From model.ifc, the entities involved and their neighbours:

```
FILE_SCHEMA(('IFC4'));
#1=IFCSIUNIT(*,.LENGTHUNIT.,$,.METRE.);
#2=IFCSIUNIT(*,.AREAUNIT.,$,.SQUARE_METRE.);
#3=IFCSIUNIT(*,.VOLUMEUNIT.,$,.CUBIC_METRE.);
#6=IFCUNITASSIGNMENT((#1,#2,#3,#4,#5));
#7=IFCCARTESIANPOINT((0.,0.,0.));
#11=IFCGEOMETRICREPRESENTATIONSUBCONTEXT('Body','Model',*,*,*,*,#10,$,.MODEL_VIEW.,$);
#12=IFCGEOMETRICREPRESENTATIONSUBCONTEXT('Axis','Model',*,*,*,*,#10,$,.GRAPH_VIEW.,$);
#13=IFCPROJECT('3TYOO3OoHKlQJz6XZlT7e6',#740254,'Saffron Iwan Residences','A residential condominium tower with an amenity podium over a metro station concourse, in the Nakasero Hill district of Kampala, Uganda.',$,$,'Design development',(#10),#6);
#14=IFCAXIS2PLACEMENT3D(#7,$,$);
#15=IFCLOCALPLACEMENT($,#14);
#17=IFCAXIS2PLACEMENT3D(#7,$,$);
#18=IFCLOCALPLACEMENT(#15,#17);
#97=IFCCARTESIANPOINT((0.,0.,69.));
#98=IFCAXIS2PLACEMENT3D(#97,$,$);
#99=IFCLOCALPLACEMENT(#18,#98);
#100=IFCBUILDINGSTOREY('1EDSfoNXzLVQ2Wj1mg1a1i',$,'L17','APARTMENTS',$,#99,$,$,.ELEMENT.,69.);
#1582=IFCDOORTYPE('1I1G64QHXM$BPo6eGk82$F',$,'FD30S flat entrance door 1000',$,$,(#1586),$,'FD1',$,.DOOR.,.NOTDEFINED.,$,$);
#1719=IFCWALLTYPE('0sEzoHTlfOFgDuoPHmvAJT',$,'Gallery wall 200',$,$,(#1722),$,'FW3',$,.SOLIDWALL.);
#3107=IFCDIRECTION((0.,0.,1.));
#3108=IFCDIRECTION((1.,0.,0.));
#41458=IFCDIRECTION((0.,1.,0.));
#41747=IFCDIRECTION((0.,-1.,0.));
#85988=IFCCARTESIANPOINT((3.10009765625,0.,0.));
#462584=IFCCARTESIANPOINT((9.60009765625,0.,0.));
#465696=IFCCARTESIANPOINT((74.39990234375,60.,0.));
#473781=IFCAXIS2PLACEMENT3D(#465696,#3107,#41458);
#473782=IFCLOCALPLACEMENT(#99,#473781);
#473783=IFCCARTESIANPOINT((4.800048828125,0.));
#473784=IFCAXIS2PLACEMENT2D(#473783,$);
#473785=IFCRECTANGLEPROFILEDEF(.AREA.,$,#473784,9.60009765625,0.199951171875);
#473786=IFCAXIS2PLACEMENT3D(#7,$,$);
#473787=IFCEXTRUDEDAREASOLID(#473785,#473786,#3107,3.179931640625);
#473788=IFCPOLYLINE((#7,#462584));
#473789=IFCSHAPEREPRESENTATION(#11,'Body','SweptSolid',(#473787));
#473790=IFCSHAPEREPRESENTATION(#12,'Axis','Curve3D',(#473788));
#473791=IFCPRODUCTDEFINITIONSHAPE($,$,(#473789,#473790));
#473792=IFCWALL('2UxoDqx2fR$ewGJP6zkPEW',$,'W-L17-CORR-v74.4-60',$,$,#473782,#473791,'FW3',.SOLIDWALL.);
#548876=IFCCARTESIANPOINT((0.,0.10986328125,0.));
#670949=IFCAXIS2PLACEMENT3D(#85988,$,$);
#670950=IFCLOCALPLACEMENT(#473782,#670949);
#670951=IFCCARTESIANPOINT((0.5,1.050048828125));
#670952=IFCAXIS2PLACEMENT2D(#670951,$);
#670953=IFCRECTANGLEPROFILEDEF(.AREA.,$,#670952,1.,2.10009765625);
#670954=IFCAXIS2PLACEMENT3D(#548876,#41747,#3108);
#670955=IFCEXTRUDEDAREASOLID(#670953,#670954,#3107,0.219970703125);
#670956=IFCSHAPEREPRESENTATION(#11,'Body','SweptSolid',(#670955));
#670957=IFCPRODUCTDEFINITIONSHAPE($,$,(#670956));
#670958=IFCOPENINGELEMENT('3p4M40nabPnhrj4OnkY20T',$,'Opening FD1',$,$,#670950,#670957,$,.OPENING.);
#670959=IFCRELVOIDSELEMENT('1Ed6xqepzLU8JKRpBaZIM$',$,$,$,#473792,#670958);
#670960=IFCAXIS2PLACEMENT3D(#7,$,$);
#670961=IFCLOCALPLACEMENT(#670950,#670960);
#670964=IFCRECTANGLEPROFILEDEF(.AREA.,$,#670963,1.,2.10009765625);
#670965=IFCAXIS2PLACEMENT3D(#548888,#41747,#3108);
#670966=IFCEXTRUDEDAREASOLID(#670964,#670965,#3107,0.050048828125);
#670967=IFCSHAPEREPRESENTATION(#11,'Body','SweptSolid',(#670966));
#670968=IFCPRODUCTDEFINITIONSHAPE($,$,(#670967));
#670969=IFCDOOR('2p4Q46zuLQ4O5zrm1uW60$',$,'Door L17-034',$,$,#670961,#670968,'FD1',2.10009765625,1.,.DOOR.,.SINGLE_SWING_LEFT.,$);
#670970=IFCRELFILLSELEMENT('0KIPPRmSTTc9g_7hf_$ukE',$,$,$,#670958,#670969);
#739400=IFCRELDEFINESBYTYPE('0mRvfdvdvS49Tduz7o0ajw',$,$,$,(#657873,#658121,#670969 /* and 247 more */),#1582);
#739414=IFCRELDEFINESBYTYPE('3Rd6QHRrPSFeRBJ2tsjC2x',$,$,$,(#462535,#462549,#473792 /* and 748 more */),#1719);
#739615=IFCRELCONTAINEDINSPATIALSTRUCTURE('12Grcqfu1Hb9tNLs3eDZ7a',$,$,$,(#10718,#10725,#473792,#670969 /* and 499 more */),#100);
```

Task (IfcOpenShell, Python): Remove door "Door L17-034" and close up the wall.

```python
import ifcopenshell
import ifcopenshell.api.feature
import ifcopenshell.api.root
import ifcopenshell.geom
import ifcopenshell.util.shape

model = ifcopenshell.open("model.ifc")
settings = ifcopenshell.geom.settings()


def volume(element):
    """Net volume in cubic metres, openings subtracted."""
    shape = ifcopenshell.geom.create_shape(settings, element)
    return ifcopenshell.util.shape.get_volume(shape.geometry)


door = model.by_guid("2p4Q46zuLQ4O5zrm1uW60$")
opening = door.FillsVoids[0].RelatingOpeningElement
wall = opening.VoidsElements[0].RelatingBuildingElement
before = volume(wall)

ifcopenshell.api.root.remove_product(model, product=door)
ifcopenshell.api.feature.remove_feature(model, feature=opening)

after = volume(wall)

print(f"wall volume {before:.3f} -> {after:.3f} m3")

model.write("model_updated.ifc")
```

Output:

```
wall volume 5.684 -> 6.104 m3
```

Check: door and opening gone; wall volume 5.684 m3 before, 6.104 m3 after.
